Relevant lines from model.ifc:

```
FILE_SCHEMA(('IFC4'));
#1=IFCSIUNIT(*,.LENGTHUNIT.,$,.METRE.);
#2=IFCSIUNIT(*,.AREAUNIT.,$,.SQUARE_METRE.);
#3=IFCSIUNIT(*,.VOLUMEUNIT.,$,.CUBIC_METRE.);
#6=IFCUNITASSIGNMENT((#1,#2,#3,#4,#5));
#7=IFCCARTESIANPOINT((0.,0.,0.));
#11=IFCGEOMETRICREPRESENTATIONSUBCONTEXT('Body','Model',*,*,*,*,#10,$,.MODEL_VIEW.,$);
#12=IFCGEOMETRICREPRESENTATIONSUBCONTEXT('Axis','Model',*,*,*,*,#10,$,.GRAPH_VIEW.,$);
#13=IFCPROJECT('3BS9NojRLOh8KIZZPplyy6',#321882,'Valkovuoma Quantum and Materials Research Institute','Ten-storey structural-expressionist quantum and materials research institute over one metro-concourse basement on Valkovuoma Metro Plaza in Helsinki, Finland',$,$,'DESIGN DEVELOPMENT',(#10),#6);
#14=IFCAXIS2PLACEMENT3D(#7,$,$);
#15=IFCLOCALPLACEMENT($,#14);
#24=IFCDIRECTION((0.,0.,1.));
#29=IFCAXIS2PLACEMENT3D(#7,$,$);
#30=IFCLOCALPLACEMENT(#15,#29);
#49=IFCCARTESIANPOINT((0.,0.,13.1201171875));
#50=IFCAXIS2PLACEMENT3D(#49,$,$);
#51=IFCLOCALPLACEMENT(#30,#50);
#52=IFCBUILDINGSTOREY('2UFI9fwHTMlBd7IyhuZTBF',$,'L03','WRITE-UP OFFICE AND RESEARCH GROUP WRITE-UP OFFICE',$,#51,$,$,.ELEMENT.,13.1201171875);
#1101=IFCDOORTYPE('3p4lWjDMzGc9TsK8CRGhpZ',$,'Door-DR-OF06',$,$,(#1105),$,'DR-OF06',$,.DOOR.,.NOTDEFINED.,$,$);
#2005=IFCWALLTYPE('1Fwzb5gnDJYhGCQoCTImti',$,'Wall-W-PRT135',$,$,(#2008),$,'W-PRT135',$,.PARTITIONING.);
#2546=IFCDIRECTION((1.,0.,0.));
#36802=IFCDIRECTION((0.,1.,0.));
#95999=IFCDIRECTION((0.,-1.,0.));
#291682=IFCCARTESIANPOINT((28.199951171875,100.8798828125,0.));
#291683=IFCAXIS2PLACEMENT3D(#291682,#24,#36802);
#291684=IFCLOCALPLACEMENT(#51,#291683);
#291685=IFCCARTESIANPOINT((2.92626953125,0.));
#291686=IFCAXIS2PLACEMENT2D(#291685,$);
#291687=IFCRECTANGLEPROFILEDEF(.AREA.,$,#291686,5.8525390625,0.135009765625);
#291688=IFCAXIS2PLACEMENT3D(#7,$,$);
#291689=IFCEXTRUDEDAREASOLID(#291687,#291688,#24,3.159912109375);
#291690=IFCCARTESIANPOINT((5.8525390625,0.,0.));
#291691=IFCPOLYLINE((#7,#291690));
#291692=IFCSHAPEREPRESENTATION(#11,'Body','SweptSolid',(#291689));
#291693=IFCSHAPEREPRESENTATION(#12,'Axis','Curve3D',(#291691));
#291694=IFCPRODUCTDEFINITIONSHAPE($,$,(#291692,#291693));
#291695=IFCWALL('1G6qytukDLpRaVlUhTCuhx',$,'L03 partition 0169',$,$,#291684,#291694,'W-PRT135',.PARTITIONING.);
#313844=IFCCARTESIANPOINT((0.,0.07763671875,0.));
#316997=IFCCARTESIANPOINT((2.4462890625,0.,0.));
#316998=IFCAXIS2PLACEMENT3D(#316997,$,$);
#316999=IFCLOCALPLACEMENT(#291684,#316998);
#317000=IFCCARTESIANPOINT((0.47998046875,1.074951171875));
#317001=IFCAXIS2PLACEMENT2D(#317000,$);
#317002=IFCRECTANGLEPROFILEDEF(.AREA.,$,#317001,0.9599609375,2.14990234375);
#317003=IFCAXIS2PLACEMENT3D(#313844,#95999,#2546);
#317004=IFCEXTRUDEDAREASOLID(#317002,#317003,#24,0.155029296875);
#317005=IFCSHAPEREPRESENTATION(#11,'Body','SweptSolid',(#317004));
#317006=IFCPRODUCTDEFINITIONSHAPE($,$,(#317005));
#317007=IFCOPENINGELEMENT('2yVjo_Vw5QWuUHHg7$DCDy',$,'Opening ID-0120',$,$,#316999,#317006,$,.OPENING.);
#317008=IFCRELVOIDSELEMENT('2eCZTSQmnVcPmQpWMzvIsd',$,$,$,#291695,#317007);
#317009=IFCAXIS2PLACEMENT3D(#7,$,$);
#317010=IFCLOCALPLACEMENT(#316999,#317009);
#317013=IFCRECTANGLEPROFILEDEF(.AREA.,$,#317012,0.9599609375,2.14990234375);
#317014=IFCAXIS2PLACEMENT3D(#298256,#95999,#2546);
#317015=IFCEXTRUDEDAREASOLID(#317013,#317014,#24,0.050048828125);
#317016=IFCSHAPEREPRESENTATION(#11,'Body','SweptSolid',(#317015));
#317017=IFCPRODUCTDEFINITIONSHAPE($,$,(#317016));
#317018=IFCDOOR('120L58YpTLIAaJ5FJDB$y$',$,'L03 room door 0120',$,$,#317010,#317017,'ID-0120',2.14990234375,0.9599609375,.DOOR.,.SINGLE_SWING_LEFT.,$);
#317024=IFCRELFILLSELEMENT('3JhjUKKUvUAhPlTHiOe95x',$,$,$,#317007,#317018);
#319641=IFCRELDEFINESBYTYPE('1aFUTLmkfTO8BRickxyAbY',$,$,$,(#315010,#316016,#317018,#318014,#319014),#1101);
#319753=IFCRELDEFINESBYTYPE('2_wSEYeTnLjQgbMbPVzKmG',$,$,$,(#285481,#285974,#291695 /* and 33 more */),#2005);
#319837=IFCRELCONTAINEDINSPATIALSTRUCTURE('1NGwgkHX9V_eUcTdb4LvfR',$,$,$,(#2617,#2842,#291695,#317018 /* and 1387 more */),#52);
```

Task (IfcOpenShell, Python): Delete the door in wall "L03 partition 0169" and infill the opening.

```python
import ifcopenshell
import ifcopenshell.api.feature
import ifcopenshell.api.root
import ifcopenshell.geom
import ifcopenshell.util.shape

model = ifcopenshell.open("model.ifc")
settings = ifcopenshell.geom.settings()


def volume(element):
    """Net volume in cubic metres, openings subtracted."""
    shape = ifcopenshell.geom.create_shape(settings, element)
    return ifcopenshell.util.shape.get_volume(shape.geometry)


door = model.by_id(317018)
opening = door.FillsVoids[0].RelatingOpeningElement
wall = opening.VoidsElements[0].RelatingBuildingElement
before = volume(wall)

ifcopenshell.api.root.remove_product(model, product=door)
ifcopenshell.api.feature.remove_feature(model, feature=opening)

after = volume(wall)

print(f"wall volume {before:.3f} -> {after:.3f} m3")

model.write("model_edited.ifc")
```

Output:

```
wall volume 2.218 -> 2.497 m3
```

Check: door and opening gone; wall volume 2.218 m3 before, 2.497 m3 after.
